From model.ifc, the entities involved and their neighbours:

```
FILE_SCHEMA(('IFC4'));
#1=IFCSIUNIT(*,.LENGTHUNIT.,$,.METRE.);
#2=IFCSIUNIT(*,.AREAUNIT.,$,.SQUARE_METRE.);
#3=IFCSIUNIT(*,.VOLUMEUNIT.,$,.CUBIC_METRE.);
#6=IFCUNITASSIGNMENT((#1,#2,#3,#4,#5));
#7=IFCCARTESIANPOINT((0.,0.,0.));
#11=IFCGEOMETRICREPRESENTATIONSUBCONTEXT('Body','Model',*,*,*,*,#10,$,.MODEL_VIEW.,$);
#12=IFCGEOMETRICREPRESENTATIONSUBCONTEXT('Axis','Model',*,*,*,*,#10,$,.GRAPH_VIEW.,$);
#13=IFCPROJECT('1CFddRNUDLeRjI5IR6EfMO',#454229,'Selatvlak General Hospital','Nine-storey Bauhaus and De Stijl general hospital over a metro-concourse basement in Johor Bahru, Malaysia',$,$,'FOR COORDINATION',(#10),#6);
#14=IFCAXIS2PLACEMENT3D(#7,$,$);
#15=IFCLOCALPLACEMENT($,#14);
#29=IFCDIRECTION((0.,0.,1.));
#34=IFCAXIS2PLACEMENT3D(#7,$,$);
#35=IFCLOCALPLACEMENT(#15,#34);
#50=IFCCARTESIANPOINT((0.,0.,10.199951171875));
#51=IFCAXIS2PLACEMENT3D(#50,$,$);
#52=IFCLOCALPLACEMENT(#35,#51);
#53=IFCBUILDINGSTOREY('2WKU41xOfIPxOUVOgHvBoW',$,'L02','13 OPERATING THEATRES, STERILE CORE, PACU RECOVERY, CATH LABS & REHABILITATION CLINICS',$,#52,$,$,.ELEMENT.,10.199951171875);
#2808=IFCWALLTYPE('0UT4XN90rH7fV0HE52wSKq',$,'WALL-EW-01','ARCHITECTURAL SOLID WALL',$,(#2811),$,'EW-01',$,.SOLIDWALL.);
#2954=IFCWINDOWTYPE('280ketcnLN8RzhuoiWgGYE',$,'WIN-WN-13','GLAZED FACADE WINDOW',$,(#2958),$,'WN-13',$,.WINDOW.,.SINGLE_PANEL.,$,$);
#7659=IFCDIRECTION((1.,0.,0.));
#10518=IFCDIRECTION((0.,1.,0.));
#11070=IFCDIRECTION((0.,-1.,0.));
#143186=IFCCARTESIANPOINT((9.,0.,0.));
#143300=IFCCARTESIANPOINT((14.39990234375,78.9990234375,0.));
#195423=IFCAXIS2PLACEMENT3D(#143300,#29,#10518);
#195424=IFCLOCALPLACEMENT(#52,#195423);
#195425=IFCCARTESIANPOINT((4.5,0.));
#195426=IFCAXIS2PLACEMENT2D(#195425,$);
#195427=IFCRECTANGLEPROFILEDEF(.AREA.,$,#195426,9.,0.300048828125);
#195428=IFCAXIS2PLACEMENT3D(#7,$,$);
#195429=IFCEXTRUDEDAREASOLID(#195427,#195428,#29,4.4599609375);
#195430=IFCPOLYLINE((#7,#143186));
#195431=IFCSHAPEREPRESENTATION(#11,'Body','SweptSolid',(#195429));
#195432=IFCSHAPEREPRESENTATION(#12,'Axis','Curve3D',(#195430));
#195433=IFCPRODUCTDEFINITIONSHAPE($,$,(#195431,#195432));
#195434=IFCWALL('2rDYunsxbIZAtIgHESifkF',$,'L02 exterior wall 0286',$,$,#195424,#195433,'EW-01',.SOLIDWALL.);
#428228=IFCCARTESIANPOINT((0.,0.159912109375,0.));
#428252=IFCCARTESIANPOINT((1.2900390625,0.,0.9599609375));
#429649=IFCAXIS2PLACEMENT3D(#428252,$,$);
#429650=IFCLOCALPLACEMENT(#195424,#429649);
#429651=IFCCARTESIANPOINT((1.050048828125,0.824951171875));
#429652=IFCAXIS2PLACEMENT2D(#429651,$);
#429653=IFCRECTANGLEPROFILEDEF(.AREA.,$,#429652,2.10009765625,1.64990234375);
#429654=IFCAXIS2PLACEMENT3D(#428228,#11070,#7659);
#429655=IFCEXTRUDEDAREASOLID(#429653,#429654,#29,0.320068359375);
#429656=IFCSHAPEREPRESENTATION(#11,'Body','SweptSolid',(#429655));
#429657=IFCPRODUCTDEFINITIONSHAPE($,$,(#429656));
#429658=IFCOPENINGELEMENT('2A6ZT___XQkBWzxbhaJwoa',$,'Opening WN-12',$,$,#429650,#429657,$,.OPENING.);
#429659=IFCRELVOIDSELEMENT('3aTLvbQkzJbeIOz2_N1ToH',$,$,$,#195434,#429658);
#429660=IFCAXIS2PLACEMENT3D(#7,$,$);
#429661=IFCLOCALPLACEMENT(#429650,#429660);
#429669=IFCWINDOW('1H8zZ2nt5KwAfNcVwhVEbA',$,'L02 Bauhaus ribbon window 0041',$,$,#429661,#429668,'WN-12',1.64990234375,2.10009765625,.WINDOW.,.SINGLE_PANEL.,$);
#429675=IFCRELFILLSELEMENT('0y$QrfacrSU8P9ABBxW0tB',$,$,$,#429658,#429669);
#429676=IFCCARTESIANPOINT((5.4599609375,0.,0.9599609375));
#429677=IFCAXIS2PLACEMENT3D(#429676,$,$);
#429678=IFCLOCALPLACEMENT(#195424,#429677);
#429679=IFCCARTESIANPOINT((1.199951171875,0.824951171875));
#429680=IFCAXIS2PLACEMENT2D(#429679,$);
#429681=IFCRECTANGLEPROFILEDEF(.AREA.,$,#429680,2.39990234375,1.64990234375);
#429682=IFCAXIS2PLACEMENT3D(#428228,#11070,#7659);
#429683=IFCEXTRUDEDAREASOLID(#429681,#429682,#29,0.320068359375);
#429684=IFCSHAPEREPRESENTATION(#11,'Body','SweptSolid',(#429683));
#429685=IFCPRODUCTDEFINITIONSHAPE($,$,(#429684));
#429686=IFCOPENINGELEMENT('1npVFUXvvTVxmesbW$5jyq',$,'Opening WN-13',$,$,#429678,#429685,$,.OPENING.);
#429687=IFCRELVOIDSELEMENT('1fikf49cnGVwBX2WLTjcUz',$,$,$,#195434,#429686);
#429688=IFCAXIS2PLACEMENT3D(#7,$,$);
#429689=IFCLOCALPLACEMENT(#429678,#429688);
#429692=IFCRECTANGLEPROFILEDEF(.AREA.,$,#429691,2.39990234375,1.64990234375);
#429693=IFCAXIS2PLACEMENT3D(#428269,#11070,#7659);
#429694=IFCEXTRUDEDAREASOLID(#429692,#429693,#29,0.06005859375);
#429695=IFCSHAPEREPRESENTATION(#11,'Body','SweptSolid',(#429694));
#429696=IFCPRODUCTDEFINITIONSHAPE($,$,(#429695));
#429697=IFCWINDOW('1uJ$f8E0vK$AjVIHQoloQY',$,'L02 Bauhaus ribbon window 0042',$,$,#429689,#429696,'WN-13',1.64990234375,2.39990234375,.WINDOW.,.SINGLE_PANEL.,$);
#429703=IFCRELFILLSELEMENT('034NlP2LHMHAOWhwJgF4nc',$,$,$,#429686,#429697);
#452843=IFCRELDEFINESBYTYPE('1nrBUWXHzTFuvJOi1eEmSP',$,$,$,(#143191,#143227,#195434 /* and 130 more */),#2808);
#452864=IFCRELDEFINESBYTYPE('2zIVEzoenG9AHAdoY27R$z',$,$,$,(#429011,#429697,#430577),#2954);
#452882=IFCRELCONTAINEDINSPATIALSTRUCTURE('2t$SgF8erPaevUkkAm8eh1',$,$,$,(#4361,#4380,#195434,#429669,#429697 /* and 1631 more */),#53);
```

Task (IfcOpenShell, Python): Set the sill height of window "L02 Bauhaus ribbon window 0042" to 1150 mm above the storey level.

```python
import numpy as np
import ifcopenshell
import ifcopenshell.api.geometry
import ifcopenshell.geom
import ifcopenshell.util.element
import ifcopenshell.util.placement
import ifcopenshell.util.shape
import ifcopenshell.util.unit

model = ifcopenshell.open("model.ifc")
unit_scale = ifcopenshell.util.unit.calculate_unit_scale(model)

window = model.by_guid("1uJ$f8E0vK$AjVIHQoloQY")
opening = window.FillsVoids[0].RelatingOpeningElement
storey = ifcopenshell.util.element.get_container(window, ifc_class="IfcBuildingStorey")
level = ifcopenshell.util.placement.get_local_placement(storey.ObjectPlacement)[2, 3]

# The opening's origin need not be at the sill, so measure its lowest point.
shape = ifcopenshell.geom.create_shape(ifcopenshell.geom.settings(), opening)
bottom = ifcopenshell.util.shape.get_shape_bottom_elevation(shape, shape.geometry) / unit_scale
dz = level + 1.15 / unit_scale - bottom

shift = np.array([0.0, 0.0, dz])
# The window is placed relative to its opening, so it follows when the opening moves.
matrix = ifcopenshell.util.placement.get_local_placement(opening.ObjectPlacement)
matrix[:3, 3] += shift
ifcopenshell.api.geometry.edit_object_placement(
    model, product=opening, matrix=matrix, is_si=False, should_transform_children=True
)

print(f"moved by {dz * unit_scale:+.3f} m")

model.write("model_updated.ifc")
```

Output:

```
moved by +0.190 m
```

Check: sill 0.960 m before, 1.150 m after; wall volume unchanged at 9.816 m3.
